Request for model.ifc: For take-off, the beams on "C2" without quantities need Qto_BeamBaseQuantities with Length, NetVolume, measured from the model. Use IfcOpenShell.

First a look at what the model holds.

```python
import ifcopenshell
import ifcopenshell.util.element
import ifcopenshell.util.unit

model = ifcopenshell.open("model.ifc")
print(model.schema)
for unit_type in ("LENGTHUNIT", "AREAUNIT", "VOLUMEUNIT"):
    print(unit_type, ifcopenshell.util.unit.calculate_unit_scale(model, unit_type))
storey = next(s for s in model.by_type("IfcBuildingStorey") if s.Name == "C2")
beams = [e for e in ifcopenshell.util.element.get_decomposition(storey) if e.is_a("IfcBeam")]
for e in sorted(beams, key=lambda e: e.id()):
    print(e.id(), e.is_a(), e.Name, list(ifcopenshell.util.element.get_psets(e, qtos_only=True)), sep=" | ")
```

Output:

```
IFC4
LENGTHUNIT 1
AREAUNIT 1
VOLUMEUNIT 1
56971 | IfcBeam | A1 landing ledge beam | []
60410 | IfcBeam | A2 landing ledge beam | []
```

```python
import ifcopenshell
import ifcopenshell.api.pset
import ifcopenshell.geom
import ifcopenshell.util.element
import ifcopenshell.util.shape
import ifcopenshell.util.unit

model = ifcopenshell.open("model.ifc")
unit_scale = ifcopenshell.util.unit.calculate_unit_scale(model)
volume_scale = ifcopenshell.util.unit.calculate_unit_scale(model, "VOLUMEUNIT")
settings = ifcopenshell.geom.settings()

storey = next(s for s in model.by_type("IfcBuildingStorey") if s.Name == "C2")
beams = [e for e in ifcopenshell.util.element.get_decomposition(storey) if e.is_a("IfcBeam")]

for e in sorted(beams, key=lambda e: e.id()):
    if ifcopenshell.util.element.get_psets(e, qtos_only=True, should_inherit=False):
        continue
    # Geometry comes back in metres, in the element's own axes.
    shape = ifcopenshell.geom.create_shape(settings, e)
    values = {
        "Length": ifcopenshell.util.shape.get_max_xyz(shape.geometry) / unit_scale,
        "NetVolume": ifcopenshell.util.shape.get_volume(shape.geometry) / volume_scale,
    }
    qto = ifcopenshell.api.pset.add_qto(model, product=e, name="Qto_BeamBaseQuantities")
    ifcopenshell.api.pset.edit_qto(model, qto=qto, properties=values)
    print(e.id(), {k: round(v, 3) for k, v in values.items()})

model.write("model_v2.ifc")
```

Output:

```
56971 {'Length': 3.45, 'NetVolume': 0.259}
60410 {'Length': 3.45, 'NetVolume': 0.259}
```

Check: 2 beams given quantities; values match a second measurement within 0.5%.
